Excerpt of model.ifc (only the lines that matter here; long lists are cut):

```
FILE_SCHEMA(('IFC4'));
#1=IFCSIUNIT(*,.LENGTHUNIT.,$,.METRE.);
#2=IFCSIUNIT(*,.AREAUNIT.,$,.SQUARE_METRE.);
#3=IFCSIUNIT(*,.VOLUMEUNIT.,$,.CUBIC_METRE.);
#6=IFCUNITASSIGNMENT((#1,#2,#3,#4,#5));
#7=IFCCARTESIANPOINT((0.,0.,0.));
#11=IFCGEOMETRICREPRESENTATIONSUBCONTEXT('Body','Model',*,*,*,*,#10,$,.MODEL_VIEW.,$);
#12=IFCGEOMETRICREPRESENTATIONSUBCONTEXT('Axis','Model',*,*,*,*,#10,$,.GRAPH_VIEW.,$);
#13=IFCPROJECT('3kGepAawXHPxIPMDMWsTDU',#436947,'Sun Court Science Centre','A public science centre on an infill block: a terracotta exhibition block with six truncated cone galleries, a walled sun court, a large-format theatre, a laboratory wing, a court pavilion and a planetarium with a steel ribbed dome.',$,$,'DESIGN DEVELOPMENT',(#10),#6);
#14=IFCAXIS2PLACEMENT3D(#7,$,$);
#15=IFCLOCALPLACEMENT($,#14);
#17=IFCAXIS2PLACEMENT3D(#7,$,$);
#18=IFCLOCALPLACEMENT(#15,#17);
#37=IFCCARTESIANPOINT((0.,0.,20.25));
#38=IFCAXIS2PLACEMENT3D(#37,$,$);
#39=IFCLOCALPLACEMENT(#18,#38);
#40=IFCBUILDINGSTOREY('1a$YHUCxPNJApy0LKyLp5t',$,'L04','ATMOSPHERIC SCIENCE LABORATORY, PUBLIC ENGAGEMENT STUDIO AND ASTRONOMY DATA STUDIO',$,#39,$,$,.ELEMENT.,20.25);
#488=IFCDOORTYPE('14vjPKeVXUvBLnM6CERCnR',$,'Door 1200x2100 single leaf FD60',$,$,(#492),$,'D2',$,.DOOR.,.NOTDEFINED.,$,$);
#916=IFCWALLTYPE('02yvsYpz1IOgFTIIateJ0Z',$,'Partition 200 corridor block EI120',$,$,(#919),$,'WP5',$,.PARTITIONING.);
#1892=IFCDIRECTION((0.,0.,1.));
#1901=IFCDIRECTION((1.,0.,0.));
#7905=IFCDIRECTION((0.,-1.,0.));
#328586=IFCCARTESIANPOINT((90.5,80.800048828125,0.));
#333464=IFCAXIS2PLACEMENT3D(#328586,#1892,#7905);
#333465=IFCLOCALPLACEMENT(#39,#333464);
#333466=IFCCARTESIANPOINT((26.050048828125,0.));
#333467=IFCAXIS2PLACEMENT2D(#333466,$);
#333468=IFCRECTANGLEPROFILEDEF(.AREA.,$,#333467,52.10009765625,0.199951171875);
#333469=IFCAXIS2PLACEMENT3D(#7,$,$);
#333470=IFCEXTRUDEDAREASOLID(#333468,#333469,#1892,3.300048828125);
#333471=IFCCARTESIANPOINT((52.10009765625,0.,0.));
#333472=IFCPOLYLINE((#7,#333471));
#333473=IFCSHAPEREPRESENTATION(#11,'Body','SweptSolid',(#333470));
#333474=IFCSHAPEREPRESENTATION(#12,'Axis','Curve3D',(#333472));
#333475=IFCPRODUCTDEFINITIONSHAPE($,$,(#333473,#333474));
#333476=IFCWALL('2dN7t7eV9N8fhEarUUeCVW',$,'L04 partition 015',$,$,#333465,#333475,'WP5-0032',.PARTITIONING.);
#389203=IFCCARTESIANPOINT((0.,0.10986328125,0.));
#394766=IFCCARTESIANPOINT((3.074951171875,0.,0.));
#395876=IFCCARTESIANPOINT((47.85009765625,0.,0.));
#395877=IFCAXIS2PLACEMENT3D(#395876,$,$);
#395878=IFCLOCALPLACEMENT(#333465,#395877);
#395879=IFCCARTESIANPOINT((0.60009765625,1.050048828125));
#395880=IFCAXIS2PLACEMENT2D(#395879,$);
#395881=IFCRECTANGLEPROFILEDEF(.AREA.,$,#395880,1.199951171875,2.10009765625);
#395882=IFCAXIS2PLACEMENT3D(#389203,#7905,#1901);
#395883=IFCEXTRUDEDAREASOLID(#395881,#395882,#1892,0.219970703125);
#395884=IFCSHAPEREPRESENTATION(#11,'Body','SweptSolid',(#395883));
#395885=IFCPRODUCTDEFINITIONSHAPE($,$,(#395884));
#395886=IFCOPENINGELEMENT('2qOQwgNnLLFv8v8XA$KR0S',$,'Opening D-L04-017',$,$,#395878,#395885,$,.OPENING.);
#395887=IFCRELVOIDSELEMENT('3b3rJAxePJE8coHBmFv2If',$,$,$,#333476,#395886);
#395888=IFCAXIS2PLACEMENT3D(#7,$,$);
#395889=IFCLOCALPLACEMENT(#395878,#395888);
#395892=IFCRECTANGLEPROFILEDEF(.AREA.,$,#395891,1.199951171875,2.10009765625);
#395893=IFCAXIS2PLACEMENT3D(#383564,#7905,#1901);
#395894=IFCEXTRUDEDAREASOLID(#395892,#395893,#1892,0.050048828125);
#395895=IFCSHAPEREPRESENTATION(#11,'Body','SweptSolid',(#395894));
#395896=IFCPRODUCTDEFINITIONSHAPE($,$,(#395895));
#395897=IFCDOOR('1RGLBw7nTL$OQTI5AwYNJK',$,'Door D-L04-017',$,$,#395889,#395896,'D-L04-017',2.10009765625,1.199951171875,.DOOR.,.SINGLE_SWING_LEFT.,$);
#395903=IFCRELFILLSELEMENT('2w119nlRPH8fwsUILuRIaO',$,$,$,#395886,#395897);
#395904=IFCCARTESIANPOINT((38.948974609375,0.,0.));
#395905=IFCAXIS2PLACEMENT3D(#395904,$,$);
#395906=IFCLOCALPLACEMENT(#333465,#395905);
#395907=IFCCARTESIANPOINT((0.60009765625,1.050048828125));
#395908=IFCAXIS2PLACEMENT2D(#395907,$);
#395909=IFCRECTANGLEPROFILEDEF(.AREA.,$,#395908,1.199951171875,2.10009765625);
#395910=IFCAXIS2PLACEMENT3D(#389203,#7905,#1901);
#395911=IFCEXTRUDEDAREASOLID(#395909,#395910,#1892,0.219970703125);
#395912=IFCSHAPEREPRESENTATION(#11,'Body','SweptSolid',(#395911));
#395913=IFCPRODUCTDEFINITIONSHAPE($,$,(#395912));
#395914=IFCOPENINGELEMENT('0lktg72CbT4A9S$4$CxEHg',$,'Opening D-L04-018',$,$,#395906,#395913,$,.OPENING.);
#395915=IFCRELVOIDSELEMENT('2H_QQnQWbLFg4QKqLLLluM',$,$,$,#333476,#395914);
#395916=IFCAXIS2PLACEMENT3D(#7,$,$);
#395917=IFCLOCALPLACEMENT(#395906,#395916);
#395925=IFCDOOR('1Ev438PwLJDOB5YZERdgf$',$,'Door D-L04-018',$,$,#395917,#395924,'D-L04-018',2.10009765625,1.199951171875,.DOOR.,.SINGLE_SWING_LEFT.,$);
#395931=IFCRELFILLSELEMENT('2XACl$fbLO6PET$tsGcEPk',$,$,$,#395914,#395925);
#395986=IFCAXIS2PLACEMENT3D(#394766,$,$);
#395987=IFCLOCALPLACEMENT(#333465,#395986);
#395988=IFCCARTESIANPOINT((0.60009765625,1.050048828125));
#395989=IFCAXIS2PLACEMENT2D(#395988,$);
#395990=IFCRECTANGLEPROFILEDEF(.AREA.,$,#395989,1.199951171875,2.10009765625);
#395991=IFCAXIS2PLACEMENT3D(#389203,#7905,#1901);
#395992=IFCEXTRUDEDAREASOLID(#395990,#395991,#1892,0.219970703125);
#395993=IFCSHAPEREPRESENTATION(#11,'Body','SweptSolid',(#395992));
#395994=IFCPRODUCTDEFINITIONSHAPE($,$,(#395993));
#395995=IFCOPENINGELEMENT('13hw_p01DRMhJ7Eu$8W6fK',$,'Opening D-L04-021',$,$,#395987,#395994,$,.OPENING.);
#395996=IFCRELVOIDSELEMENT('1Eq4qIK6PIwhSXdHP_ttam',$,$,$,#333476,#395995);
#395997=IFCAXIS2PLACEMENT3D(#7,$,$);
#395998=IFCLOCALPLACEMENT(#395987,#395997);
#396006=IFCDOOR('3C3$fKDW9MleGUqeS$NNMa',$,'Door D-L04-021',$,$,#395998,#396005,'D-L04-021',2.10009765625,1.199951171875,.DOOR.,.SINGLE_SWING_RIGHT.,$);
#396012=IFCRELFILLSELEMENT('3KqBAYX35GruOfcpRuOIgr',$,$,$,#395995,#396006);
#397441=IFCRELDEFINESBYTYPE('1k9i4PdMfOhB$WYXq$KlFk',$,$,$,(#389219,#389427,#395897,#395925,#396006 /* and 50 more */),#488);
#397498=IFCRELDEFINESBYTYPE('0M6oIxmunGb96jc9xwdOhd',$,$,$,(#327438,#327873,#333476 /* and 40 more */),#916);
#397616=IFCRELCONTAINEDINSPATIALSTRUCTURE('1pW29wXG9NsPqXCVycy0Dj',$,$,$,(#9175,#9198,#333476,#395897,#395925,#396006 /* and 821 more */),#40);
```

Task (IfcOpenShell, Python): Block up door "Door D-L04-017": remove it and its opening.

```python
import ifcopenshell
import ifcopenshell.api.feature
import ifcopenshell.api.root
import ifcopenshell.geom
import ifcopenshell.util.shape

model = ifcopenshell.open("model.ifc")
settings = ifcopenshell.geom.settings()


def volume(element):
    """Net volume in cubic metres, openings subtracted."""
    shape = ifcopenshell.geom.create_shape(settings, element)
    return ifcopenshell.util.shape.get_volume(shape.geometry)


door = model.by_guid("1RGLBw7nTL$OQTI5AwYNJK")
opening = door.FillsVoids[0].RelatingOpeningElement
wall = opening.VoidsElements[0].RelatingBuildingElement
before = volume(wall)

ifcopenshell.api.root.remove_product(model, product=door)
ifcopenshell.api.feature.remove_feature(model, feature=opening)

after = volume(wall)

print(f"wall volume {before:.3f} -> {after:.3f} m3")

model.write("model_rev.ifc")
```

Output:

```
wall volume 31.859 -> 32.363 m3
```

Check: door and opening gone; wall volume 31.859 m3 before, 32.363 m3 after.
